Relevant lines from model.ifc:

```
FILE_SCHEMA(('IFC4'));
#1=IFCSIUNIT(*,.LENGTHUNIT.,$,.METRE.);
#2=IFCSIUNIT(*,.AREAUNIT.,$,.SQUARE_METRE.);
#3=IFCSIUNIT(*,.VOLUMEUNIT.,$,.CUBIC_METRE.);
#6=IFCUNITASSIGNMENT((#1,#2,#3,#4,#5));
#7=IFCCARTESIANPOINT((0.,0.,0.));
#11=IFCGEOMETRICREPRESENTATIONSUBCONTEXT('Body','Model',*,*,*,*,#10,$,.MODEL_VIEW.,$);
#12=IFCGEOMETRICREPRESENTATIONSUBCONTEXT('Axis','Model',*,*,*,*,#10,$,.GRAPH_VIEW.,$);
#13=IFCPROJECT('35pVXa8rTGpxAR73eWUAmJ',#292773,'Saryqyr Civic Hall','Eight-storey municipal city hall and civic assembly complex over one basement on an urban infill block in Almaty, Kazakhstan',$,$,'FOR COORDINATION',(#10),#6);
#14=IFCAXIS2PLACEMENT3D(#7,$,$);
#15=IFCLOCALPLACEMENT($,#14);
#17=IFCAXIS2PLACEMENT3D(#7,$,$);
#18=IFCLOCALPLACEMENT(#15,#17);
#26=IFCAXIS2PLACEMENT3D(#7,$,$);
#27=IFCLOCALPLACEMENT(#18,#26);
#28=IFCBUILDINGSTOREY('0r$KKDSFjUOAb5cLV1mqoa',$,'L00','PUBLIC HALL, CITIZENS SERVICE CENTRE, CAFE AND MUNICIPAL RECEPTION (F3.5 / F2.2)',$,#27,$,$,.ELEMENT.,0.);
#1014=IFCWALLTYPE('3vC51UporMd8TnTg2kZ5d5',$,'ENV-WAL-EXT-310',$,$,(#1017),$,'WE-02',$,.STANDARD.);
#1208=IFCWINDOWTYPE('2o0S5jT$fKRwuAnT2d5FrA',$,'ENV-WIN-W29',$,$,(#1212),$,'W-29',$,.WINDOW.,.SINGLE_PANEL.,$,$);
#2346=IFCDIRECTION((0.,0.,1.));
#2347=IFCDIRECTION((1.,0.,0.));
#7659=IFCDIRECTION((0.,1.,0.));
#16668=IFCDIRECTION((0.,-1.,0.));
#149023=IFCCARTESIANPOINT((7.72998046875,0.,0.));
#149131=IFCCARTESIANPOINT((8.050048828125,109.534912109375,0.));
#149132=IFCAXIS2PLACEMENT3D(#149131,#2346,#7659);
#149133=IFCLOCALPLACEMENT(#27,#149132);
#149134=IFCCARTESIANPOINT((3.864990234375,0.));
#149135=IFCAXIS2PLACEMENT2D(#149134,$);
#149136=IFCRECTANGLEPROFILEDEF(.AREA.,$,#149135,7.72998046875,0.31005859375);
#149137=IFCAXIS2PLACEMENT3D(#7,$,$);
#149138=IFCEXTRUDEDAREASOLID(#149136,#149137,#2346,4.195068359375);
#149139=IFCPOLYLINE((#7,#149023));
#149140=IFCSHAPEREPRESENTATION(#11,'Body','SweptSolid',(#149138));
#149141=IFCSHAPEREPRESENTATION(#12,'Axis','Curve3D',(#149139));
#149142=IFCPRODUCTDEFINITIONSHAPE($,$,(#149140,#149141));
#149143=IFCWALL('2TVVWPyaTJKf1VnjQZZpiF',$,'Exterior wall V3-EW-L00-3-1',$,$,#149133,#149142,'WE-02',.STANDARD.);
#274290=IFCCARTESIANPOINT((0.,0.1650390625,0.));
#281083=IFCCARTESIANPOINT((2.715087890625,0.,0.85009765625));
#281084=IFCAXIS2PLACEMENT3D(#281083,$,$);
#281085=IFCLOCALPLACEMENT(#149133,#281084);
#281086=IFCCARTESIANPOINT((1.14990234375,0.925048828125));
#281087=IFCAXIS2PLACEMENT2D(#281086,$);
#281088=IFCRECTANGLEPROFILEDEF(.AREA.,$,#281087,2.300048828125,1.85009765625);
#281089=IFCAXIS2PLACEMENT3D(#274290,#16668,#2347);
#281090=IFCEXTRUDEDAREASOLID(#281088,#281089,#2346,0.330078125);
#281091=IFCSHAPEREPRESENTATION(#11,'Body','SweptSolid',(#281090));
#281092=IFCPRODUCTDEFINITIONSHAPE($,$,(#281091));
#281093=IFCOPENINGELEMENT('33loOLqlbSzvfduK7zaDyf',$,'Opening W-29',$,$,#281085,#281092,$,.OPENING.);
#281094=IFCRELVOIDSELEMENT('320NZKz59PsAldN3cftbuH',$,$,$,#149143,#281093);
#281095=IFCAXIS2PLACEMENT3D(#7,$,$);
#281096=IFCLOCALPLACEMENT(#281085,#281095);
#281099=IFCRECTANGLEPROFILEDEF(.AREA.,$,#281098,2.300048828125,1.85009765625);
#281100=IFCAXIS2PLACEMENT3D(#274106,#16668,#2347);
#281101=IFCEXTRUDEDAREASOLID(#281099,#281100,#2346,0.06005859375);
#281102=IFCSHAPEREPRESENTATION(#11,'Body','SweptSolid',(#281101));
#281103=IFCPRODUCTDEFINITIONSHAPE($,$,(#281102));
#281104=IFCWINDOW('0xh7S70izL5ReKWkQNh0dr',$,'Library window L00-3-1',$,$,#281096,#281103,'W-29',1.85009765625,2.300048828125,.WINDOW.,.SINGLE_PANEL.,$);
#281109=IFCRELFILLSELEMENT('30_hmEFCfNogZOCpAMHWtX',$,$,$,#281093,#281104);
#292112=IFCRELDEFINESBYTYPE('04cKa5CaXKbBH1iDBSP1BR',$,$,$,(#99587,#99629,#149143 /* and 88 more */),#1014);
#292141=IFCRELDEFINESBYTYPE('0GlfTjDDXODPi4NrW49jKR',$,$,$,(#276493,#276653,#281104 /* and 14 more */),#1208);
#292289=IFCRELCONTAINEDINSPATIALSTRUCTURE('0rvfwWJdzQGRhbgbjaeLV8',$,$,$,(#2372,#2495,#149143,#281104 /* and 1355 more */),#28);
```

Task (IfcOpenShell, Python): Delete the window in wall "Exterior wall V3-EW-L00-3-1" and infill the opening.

```python
import ifcopenshell
import ifcopenshell.api.feature
import ifcopenshell.api.root
import ifcopenshell.geom
import ifcopenshell.util.shape

model = ifcopenshell.open("model.ifc")
settings = ifcopenshell.geom.settings()


def volume(element):
    """Net volume in cubic metres, openings subtracted."""
    shape = ifcopenshell.geom.create_shape(settings, element)
    return ifcopenshell.util.shape.get_volume(shape.geometry)


window = model.by_guid("0xh7S70izL5ReKWkQNh0dr")
opening = window.FillsVoids[0].RelatingOpeningElement
wall = opening.VoidsElements[0].RelatingBuildingElement
before = volume(wall)

ifcopenshell.api.root.remove_product(model, product=window)
ifcopenshell.api.feature.remove_feature(model, feature=opening)

after = volume(wall)

print(f"wall volume {before:.3f} -> {after:.3f} m3")

model.write("model_updated.ifc")
```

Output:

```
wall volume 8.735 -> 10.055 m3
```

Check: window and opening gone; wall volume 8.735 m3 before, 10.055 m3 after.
